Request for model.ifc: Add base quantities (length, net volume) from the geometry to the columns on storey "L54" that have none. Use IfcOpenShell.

First a look at what the model holds.

```python
import ifcopenshell
import ifcopenshell.util.element
import ifcopenshell.util.unit

model = ifcopenshell.open("model.ifc")
print(model.schema)
for unit_type in ("LENGTHUNIT", "AREAUNIT", "VOLUMEUNIT"):
    print(unit_type, ifcopenshell.util.unit.calculate_unit_scale(model, unit_type))
storey = next(s for s in model.by_type("IfcBuildingStorey") if s.Name == "L54")
columns = [e for e in ifcopenshell.util.element.get_decomposition(storey) if e.is_a("IfcColumn")]
for e in sorted(columns, key=lambda e: e.id()):
    print(e.id(), e.is_a(), e.Name, list(ifcopenshell.util.element.get_psets(e, qtos_only=True)), sep=" | ")
```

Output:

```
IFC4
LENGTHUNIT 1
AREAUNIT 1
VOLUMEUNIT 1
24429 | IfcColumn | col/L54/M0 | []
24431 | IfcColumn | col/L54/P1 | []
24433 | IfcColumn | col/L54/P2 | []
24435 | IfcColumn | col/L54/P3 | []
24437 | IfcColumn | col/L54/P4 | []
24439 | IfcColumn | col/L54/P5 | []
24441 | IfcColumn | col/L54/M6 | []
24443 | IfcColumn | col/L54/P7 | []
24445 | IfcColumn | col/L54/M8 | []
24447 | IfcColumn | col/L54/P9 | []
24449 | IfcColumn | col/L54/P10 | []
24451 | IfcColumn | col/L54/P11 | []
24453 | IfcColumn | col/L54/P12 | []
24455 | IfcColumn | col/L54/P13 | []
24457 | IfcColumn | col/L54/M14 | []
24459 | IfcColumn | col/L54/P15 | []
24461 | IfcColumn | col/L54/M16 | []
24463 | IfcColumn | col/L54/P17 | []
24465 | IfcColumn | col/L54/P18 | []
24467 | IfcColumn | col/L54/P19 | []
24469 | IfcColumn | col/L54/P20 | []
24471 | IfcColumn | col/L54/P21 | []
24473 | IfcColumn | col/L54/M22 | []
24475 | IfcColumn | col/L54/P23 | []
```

```python
import ifcopenshell
import ifcopenshell.api.pset
import ifcopenshell.geom
import ifcopenshell.util.element
import ifcopenshell.util.shape
import ifcopenshell.util.unit

model = ifcopenshell.open("model.ifc")
unit_scale = ifcopenshell.util.unit.calculate_unit_scale(model)
volume_scale = ifcopenshell.util.unit.calculate_unit_scale(model, "VOLUMEUNIT")
settings = ifcopenshell.geom.settings()

storey = next(s for s in model.by_type("IfcBuildingStorey") if s.Name == "L54")
columns = [e for e in ifcopenshell.util.element.get_decomposition(storey) if e.is_a("IfcColumn")]

for e in sorted(columns, key=lambda e: e.id()):
    if ifcopenshell.util.element.get_psets(e, qtos_only=True, should_inherit=False):
        continue
    # Geometry comes back in metres, in the element's own axes.
    shape = ifcopenshell.geom.create_shape(settings, e)
    values = {
        "Length": ifcopenshell.util.shape.get_z(shape.geometry) / unit_scale,
        "NetVolume": ifcopenshell.util.shape.get_volume(shape.geometry) / volume_scale,
    }
    qto = ifcopenshell.api.pset.add_qto(model, product=e, name="Qto_ColumnBaseQuantities")
    ifcopenshell.api.pset.edit_qto(model, qto=qto, properties=values)
    print(e.id(), {k: round(v, 3) for k, v in values.items()})

model.write("model_rev.ifc")
```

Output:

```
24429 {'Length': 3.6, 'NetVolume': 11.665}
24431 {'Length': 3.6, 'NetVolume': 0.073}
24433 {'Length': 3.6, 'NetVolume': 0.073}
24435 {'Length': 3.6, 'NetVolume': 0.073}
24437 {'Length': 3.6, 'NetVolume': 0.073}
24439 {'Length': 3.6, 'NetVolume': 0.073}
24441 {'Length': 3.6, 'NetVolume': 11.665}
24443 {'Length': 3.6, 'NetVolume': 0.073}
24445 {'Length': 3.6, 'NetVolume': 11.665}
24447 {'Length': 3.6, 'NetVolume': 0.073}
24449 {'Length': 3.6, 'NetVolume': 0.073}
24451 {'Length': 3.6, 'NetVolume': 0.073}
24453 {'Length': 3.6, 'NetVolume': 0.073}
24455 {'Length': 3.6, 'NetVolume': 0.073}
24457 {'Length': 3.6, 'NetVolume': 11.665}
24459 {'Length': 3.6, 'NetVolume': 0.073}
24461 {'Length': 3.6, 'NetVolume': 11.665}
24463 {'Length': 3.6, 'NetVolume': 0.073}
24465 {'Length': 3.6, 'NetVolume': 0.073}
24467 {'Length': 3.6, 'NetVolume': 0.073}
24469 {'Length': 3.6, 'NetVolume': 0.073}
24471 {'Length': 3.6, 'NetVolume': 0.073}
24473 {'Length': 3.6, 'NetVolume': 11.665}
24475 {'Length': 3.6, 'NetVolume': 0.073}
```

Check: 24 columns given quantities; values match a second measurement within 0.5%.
